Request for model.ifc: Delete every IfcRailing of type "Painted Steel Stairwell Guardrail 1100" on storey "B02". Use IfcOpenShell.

First a look at what the model holds.

```python
import ifcopenshell
import ifcopenshell.util.element

model = ifcopenshell.open("model.ifc")
print(model.schema)
storey = next(s for s in model.by_type("IfcBuildingStorey") if s.Name == "B02")
railings = [e for e in ifcopenshell.util.element.get_decomposition(storey) if e.is_a("IfcRailing")]
seen = {}
for e in railings:
    element_type = ifcopenshell.util.element.get_type(e)
    name = element_type.Name if element_type not in (None, e) else None
    seen[name] = seen.get(name, 0) + 1
for name, count in sorted(seen.items(), key=str):
    print(count, "x", name)
```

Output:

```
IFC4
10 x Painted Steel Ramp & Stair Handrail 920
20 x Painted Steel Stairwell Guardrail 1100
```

```python
import ifcopenshell
import ifcopenshell.api.root
import ifcopenshell.util.element

model = ifcopenshell.open("model.ifc")

storey = next(s for s in model.by_type("IfcBuildingStorey") if s.Name == "B02")
railings = [e for e in ifcopenshell.util.element.get_decomposition(storey) if e.is_a("IfcRailing")]
targets = [e for e in railings if (t := ifcopenshell.util.element.get_type(e)) not in (None, e) and t.Name == "Painted Steel Stairwell Guardrail 1100"]

for e in targets:
    ifcopenshell.api.root.remove_product(model, product=e)
print(len(targets), "removed")

model.write("model_rev.ifc")
```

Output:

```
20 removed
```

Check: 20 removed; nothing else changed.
